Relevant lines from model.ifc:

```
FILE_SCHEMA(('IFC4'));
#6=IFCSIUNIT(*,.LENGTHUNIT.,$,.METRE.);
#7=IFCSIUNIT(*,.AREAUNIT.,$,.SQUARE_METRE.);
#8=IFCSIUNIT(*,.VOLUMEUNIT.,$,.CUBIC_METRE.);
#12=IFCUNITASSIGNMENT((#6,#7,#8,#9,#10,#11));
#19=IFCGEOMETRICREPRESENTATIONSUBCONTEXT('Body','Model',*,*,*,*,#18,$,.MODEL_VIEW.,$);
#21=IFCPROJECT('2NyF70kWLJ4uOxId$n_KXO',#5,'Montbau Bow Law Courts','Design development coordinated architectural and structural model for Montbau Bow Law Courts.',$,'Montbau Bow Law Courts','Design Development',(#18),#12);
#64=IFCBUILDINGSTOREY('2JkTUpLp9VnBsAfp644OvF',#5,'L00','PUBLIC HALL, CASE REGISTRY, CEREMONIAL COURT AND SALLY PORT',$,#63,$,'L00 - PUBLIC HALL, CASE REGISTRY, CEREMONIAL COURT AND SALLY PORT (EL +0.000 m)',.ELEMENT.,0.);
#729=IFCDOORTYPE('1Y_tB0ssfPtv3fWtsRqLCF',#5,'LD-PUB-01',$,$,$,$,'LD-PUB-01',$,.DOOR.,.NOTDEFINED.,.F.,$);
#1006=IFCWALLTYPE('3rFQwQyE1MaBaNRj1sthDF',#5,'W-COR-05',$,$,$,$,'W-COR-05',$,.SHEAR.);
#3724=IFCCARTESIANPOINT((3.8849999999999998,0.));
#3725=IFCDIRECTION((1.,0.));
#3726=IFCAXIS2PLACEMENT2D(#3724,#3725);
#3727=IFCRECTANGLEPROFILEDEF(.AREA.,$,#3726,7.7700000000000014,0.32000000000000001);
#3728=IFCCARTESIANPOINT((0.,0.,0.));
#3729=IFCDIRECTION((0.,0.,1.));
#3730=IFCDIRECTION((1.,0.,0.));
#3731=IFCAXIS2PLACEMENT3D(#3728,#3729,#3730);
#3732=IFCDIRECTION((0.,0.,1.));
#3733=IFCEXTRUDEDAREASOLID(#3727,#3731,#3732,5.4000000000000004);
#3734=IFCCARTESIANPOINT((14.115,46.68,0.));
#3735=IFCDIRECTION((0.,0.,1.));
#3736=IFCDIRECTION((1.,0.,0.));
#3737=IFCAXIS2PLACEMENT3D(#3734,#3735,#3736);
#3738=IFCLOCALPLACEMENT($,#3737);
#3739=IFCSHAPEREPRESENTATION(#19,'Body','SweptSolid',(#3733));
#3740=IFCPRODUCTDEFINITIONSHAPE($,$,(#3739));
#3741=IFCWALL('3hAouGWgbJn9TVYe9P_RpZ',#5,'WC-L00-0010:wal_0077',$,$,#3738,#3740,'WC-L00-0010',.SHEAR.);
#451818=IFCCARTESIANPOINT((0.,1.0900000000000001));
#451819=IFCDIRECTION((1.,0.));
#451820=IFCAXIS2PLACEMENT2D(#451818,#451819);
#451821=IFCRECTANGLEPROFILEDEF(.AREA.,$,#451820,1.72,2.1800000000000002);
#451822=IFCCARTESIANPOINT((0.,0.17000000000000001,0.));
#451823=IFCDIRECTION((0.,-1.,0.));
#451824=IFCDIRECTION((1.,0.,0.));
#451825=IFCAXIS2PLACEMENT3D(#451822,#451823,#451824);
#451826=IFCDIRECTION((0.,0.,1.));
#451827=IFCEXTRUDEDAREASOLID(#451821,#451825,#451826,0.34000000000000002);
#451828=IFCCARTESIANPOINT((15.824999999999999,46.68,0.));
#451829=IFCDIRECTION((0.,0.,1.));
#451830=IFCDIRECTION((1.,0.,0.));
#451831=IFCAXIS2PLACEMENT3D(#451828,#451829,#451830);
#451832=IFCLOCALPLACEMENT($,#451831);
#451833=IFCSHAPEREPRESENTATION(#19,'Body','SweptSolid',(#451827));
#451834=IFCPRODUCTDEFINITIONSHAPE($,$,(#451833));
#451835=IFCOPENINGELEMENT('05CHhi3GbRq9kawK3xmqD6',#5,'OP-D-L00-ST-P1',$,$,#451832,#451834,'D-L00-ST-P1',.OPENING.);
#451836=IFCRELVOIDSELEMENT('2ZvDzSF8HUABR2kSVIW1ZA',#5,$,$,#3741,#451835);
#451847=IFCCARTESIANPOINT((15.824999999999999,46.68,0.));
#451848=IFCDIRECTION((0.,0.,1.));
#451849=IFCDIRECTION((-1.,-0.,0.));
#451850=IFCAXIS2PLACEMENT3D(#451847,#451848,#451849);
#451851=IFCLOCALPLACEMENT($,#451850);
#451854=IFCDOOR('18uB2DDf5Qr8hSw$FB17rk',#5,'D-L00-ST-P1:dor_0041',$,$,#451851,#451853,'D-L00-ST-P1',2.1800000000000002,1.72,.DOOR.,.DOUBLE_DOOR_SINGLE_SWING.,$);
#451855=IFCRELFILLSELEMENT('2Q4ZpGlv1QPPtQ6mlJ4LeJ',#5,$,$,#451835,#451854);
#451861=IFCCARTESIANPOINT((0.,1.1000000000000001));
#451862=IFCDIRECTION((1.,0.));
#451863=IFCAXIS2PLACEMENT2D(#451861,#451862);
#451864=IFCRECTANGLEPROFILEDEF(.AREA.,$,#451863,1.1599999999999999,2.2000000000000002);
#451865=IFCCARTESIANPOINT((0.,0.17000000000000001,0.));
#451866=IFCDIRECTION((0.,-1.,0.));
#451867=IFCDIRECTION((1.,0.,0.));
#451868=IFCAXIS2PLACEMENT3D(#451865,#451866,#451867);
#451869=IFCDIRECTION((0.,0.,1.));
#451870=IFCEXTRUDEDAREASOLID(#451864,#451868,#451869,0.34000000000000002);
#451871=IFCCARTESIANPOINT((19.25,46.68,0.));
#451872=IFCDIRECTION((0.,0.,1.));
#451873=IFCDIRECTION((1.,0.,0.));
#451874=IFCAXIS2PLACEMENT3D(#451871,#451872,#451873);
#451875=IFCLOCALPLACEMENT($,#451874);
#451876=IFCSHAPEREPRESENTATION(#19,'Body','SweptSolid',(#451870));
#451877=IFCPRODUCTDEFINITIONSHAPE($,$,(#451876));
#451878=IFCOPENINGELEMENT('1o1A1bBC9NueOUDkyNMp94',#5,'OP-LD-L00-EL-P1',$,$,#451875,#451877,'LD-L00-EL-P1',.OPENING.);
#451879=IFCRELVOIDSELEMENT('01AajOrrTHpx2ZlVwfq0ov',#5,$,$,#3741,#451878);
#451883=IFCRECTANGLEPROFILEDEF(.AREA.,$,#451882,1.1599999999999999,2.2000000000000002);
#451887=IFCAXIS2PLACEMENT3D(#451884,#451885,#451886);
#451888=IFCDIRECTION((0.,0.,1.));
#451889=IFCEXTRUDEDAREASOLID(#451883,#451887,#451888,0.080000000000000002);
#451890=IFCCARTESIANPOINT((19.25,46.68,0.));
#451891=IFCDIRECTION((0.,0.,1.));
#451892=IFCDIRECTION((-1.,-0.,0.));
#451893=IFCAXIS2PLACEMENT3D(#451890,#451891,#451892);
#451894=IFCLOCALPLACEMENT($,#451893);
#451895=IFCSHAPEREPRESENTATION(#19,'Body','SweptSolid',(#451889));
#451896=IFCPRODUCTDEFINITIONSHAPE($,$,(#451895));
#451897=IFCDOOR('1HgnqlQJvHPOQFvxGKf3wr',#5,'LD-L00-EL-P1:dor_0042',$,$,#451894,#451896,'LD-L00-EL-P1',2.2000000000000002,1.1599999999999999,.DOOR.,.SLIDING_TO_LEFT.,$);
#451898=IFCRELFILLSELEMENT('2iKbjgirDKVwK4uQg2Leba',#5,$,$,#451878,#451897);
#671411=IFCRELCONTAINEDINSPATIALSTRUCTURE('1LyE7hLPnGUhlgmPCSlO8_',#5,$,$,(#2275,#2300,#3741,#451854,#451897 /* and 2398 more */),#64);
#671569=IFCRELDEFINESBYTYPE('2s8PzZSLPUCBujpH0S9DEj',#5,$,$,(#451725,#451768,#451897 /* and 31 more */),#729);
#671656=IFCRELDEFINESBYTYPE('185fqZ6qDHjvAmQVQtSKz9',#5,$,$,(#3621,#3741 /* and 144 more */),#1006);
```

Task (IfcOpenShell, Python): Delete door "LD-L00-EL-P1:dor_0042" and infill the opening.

```python
import ifcopenshell
import ifcopenshell.api.feature
import ifcopenshell.api.root
import ifcopenshell.geom
import ifcopenshell.util.shape

model = ifcopenshell.open("model.ifc")
settings = ifcopenshell.geom.settings()


def volume(element):
    """Net volume in cubic metres, openings subtracted."""
    shape = ifcopenshell.geom.create_shape(settings, element)
    return ifcopenshell.util.shape.get_volume(shape.geometry)


door = model.by_guid("1HgnqlQJvHPOQFvxGKf3wr")
opening = door.FillsVoids[0].RelatingOpeningElement
wall = opening.VoidsElements[0].RelatingBuildingElement
before = volume(wall)

ifcopenshell.api.root.remove_product(model, product=door)
ifcopenshell.api.feature.remove_feature(model, feature=opening)

after = volume(wall)

print(f"wall volume {before:.3f} -> {after:.3f} m3")

model.write("model-out.ifc")
```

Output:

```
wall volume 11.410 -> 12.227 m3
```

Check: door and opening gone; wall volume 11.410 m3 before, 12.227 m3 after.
